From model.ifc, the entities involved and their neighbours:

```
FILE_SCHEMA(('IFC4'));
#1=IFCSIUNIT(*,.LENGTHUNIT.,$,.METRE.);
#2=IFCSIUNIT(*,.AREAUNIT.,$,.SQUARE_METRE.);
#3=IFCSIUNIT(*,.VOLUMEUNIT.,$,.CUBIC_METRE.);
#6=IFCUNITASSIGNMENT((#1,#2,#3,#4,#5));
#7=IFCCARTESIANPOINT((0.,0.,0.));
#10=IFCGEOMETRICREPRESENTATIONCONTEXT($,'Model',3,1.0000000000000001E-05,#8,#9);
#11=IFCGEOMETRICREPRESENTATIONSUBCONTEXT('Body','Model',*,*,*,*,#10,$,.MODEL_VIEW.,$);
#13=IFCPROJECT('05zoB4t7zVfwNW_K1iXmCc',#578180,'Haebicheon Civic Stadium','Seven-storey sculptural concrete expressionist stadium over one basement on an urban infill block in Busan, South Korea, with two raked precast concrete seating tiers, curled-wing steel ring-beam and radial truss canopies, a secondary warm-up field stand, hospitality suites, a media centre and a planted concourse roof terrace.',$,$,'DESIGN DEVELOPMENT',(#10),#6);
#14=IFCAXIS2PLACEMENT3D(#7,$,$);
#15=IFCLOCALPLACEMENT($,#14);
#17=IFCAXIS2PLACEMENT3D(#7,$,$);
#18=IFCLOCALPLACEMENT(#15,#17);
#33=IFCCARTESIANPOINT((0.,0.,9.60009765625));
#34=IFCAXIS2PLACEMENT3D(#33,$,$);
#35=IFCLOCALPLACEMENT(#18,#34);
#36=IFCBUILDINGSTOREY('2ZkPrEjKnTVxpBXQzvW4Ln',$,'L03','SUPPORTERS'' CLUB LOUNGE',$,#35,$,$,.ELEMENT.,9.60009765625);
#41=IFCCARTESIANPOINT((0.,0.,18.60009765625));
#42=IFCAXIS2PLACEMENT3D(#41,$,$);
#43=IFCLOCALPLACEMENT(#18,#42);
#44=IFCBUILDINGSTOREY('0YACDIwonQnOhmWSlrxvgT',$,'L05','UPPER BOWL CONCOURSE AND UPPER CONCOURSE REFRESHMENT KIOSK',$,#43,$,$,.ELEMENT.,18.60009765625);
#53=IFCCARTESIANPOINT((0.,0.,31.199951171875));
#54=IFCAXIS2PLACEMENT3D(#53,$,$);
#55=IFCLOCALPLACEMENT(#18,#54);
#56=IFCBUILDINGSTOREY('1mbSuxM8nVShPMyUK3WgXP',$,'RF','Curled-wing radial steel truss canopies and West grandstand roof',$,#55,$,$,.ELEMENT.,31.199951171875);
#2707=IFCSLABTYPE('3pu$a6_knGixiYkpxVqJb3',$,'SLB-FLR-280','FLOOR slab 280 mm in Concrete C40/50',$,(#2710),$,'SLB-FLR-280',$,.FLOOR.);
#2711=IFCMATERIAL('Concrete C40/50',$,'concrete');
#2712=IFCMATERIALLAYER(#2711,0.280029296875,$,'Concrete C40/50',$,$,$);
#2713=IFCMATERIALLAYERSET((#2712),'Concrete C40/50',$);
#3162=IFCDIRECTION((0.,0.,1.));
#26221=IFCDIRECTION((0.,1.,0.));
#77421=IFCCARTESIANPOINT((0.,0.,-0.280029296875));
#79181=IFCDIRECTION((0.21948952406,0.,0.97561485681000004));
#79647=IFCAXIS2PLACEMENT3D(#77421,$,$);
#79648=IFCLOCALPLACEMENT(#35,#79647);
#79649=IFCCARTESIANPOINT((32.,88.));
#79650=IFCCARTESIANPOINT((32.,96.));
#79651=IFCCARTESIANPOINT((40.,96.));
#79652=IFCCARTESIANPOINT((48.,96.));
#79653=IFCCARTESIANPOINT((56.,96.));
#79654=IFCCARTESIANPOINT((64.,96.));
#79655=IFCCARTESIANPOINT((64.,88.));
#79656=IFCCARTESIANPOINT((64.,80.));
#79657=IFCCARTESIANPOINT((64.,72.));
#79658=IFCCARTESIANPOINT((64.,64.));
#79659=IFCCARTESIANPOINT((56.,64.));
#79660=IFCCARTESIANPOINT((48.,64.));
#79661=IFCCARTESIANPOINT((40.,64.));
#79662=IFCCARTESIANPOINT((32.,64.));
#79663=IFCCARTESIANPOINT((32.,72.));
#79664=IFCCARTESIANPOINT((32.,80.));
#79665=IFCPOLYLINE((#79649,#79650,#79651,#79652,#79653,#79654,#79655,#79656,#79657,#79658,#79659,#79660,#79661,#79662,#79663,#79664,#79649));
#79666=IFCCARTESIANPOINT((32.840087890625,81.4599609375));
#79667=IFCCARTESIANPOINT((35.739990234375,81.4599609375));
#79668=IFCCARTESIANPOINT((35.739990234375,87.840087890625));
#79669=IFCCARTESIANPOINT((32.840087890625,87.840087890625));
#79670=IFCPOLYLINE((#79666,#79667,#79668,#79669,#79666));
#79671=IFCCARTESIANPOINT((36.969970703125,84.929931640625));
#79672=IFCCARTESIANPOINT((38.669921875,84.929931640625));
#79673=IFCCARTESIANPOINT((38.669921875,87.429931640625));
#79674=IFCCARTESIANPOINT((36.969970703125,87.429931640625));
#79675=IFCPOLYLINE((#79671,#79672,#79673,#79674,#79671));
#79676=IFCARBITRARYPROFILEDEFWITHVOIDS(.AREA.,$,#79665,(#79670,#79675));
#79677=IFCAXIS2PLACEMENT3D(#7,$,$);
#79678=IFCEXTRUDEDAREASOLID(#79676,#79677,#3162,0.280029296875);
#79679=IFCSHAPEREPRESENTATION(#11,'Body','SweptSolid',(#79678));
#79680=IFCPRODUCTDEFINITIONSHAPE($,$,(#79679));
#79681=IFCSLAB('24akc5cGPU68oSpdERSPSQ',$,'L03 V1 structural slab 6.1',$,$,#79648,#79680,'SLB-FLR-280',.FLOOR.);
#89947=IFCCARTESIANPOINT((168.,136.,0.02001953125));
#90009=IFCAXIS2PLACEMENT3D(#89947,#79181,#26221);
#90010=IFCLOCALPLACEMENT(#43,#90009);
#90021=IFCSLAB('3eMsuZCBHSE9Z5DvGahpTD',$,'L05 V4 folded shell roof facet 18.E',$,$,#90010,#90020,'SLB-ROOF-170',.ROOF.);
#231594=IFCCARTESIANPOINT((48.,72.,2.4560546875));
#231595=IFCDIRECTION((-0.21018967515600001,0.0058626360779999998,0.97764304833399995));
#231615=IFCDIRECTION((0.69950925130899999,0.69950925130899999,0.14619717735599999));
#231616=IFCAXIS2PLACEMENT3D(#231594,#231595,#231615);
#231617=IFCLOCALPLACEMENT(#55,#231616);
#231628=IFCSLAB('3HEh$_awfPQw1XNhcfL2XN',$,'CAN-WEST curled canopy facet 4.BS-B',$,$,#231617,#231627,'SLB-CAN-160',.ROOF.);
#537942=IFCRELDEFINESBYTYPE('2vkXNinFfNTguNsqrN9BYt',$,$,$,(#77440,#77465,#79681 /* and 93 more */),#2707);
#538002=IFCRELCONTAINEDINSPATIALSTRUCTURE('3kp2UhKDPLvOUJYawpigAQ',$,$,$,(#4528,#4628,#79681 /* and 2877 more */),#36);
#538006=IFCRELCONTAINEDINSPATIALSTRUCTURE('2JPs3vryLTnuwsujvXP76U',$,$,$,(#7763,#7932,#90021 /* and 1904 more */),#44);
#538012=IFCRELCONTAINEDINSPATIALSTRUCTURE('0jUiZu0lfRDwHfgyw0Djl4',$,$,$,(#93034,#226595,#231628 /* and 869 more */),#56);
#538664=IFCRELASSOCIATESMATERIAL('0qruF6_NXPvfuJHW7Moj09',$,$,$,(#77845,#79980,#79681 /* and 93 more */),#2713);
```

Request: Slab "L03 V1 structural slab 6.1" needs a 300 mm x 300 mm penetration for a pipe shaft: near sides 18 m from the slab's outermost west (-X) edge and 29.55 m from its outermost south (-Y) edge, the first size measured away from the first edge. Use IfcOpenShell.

```python
import numpy as np
import ifcopenshell
import ifcopenshell.api.feature
import ifcopenshell.api.geometry
import ifcopenshell.api.root
import ifcopenshell.geom
import ifcopenshell.util.placement
import ifcopenshell.util.representation
import ifcopenshell.util.shape
import ifcopenshell.util.unit

model = ifcopenshell.open("model.ifc")
unit_scale = ifcopenshell.util.unit.calculate_unit_scale(model)
settings = ifcopenshell.geom.settings()


def volume(element):
    """Net volume in cubic metres, openings subtracted."""
    shape = ifcopenshell.geom.create_shape(settings, element)
    return ifcopenshell.util.shape.get_volume(shape.geometry)


slab = model.by_guid("24akc5cGPU68oSpdERSPSQ")
before = volume(slab)

# Extent in the slab's own axes, in metres. The edges named are its -X and -Y sides.
slab_shape = ifcopenshell.geom.create_shape(settings, slab)
vertices = ifcopenshell.util.shape.get_vertices(slab_shape.geometry)
x_min, y_min, bottom = vertices.min(axis=0)
top = vertices[:, 2].max()

opening = ifcopenshell.api.root.create_entity(model, ifc_class="IfcOpeningElement", name="Pipe shaft opening", predefined_type="OPENING")
context = ifcopenshell.util.representation.get_context(model, "Model", "Body", "MODEL_VIEW")
width, depth = 0.3, 0.3
outline = [(0.0, 0.0), (width, 0.0), (width, depth), (0.0, depth), (0.0, 0.0)]
# Overshoot both faces by 50 mm so the cut is clean.
shape = ifcopenshell.api.geometry.add_slab_representation(
    model, context=context, depth=top - bottom + 0.1, polyline=outline
)
ifcopenshell.api.geometry.assign_representation(model, product=opening, representation=shape)

matrix = ifcopenshell.util.placement.get_local_placement(slab.ObjectPlacement)
matrix[:, 3] = matrix @ np.append(np.array([x_min + 18, y_min + 29.55, bottom - 0.05]) / unit_scale, 1.0)
ifcopenshell.api.geometry.edit_object_placement(model, product=opening, matrix=matrix, is_si=False)
ifcopenshell.api.feature.add_feature(model, feature=opening, element=slab)

after = volume(slab)

print(f"slab volume {before:.3f} -> {after:.3f} m3")

model.write("model_updated.ifc")
```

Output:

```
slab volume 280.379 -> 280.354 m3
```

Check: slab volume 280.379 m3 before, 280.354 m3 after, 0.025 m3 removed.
